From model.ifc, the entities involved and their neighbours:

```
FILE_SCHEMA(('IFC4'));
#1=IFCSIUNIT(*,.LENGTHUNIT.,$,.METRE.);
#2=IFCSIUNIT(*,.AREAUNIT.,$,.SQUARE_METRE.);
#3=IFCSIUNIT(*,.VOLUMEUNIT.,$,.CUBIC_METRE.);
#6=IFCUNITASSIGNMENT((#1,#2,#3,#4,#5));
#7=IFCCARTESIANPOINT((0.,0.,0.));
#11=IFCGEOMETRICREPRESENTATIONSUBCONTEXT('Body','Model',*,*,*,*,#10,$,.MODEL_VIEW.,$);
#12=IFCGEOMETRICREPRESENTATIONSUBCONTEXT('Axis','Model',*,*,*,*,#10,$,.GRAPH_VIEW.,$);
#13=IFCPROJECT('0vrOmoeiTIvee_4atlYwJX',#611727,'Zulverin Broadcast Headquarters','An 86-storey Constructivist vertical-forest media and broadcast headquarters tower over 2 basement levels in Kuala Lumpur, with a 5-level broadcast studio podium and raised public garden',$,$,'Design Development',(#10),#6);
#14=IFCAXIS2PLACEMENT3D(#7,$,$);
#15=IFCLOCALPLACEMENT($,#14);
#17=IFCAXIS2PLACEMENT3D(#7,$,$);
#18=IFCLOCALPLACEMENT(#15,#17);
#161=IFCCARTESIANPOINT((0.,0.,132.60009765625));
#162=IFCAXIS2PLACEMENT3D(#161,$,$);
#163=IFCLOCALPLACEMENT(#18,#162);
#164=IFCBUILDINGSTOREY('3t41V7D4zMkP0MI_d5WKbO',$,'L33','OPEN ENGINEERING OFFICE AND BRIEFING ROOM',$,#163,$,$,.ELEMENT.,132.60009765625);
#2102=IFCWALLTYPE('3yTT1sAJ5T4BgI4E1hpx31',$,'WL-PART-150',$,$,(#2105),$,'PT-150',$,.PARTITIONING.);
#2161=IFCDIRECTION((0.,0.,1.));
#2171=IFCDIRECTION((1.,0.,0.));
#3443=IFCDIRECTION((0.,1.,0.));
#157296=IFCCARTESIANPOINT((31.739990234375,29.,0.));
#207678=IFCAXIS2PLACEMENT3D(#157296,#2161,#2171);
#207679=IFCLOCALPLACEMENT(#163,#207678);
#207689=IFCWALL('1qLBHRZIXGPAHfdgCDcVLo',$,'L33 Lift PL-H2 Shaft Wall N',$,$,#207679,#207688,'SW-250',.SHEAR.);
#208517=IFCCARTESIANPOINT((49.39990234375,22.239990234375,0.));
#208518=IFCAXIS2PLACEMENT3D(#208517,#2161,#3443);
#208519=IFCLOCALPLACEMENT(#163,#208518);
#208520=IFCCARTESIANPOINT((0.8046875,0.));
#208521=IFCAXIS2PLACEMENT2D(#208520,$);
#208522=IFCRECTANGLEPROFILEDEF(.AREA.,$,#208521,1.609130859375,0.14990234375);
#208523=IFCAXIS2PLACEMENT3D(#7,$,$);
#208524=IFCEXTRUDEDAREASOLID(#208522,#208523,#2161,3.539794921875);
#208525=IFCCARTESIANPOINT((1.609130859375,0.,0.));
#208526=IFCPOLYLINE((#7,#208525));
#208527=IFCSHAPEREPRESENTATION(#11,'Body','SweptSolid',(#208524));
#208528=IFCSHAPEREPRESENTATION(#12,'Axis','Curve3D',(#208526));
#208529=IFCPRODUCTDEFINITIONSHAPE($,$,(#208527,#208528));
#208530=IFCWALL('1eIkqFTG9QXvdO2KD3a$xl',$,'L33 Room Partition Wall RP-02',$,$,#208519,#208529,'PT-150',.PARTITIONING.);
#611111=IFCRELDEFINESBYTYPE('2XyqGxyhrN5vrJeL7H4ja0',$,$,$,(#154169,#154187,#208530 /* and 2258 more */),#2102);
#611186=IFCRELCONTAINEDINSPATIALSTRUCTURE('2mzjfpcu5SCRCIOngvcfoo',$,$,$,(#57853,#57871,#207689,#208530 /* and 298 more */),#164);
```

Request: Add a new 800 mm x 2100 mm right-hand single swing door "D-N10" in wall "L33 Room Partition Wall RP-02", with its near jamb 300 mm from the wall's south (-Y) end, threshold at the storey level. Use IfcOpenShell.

```python
import numpy as np
import ifcopenshell
import ifcopenshell.api.feature
import ifcopenshell.api.geometry
import ifcopenshell.api.root
import ifcopenshell.api.spatial
import ifcopenshell.geom
import ifcopenshell.util.element
import ifcopenshell.util.placement
import ifcopenshell.util.representation
import ifcopenshell.util.shape
import ifcopenshell.util.unit

model = ifcopenshell.open("model.ifc")
unit_scale = ifcopenshell.util.unit.calculate_unit_scale(model)
settings = ifcopenshell.geom.settings()


def volume(element):
    """Net volume in cubic metres, openings subtracted."""
    shape = ifcopenshell.geom.create_shape(settings, element)
    return ifcopenshell.util.shape.get_volume(shape.geometry)


wall = model.by_guid("1eIkqFTG9QXvdO2KD3a$xl")
storey = ifcopenshell.util.element.get_container(wall, ifc_class="IfcBuildingStorey")
context = ifcopenshell.util.representation.get_context(model, "Model", "Body", "MODEL_VIEW")
before = volume(wall)

width, height, from_end, sill = 0.8, 2.1, 0.3, 0.0  # metres

# The wall runs along its own X axis, and the end named is its -X end.
wall_shape = ifcopenshell.geom.create_shape(settings, wall)
x, y, z = ifcopenshell.util.shape.get_vertices(wall_shape.geometry).T
start = x.min() + from_end
face, thickness = float(y.min()), float(y.max() - y.min())
wall_matrix = ifcopenshell.util.placement.get_local_placement(wall.ObjectPlacement)
level = ifcopenshell.util.placement.get_local_placement(storey.ObjectPlacement)[2, 3]


def in_wall(x, y):
    """Placement at x, y metres in the wall's axes, at sill height."""
    matrix = wall_matrix.copy()
    matrix[:, 3] = wall_matrix @ np.array([x / unit_scale, y / unit_scale, 0.0, 1.0])
    matrix[2, 3] = level + sill / unit_scale
    return matrix


# Opening: a box that overshoots both wall faces by 50 mm.
opening = ifcopenshell.api.root.create_entity(model, ifc_class="IfcOpeningElement", predefined_type="OPENING")
box = ifcopenshell.api.geometry.add_wall_representation(
    model, context=context, length=width, height=height, thickness=thickness + 0.1
)
ifcopenshell.api.geometry.assign_representation(model, product=opening, representation=box)
ifcopenshell.api.geometry.edit_object_placement(model, product=opening, matrix=in_wall(start, face - 0.05), is_si=False)
ifcopenshell.api.feature.add_feature(model, feature=opening, element=wall)

door = ifcopenshell.api.root.create_entity(model, ifc_class="IfcDoor", name="D-N10", predefined_type="DOOR")
door.OverallWidth, door.OverallHeight = width / unit_scale, height / unit_scale
door.OperationType = "SINGLE_SWING_RIGHT"
body = ifcopenshell.api.geometry.add_door_representation(
    model,
    context=context,
    overall_width=door.OverallWidth,
    overall_height=door.OverallHeight,
    operation_type="SINGLE_SWING_RIGHT",
    lining_properties={"LiningDepth": thickness / unit_scale, "ThresholdDepth": thickness / unit_scale},
)
ifcopenshell.api.geometry.assign_representation(model, product=door, representation=body)
ifcopenshell.api.spatial.assign_container(model, products=[door], relating_structure=storey)
ifcopenshell.api.feature.add_filling(model, opening=opening, element=door)

# The lining spans the wall, so the door starts at the wall face.
ifcopenshell.api.geometry.edit_object_placement(model, product=door, matrix=in_wall(start, face), is_si=False)

after = volume(wall)

print(f"wall volume {before:.3f} -> {after:.3f} m3")

model.write("model-out.ifc")
```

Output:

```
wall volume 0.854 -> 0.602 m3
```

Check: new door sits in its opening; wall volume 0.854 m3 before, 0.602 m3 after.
